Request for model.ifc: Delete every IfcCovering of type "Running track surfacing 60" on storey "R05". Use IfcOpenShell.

First a look at what the model holds.

```python
import ifcopenshell
import ifcopenshell.util.element

model = ifcopenshell.open("model.ifc")
print(model.schema)
storey = next(s for s in model.by_type("IfcBuildingStorey") if s.Name == "R05")
coverings = [e for e in ifcopenshell.util.element.get_decomposition(storey) if e.is_a("IfcCovering")]
seen = {}
for e in coverings:
    element_type = ifcopenshell.util.element.get_type(e)
    name = element_type.Name if element_type not in (None, e) else None
    seen[name] = seen.get(name, 0) + 1
for name, count in sorted(seen.items(), key=str):
    print(count, "x", name)
```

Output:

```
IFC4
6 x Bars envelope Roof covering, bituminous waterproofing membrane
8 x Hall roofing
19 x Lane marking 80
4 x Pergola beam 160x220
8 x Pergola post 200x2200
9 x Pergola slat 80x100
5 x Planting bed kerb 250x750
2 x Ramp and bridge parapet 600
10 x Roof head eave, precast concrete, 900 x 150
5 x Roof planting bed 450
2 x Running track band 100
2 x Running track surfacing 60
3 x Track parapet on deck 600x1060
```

```python
import ifcopenshell
import ifcopenshell.api.root
import ifcopenshell.util.element

model = ifcopenshell.open("model.ifc")

storey = next(s for s in model.by_type("IfcBuildingStorey") if s.Name == "R05")
coverings = [e for e in ifcopenshell.util.element.get_decomposition(storey) if e.is_a("IfcCovering")]
targets = [e for e in coverings if (t := ifcopenshell.util.element.get_type(e)) not in (None, e) and t.Name == "Running track surfacing 60"]

for e in targets:
    ifcopenshell.api.root.remove_product(model, product=e)
print(len(targets), "removed")

model.write("model_edited.ifc")
```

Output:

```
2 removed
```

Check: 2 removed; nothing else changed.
